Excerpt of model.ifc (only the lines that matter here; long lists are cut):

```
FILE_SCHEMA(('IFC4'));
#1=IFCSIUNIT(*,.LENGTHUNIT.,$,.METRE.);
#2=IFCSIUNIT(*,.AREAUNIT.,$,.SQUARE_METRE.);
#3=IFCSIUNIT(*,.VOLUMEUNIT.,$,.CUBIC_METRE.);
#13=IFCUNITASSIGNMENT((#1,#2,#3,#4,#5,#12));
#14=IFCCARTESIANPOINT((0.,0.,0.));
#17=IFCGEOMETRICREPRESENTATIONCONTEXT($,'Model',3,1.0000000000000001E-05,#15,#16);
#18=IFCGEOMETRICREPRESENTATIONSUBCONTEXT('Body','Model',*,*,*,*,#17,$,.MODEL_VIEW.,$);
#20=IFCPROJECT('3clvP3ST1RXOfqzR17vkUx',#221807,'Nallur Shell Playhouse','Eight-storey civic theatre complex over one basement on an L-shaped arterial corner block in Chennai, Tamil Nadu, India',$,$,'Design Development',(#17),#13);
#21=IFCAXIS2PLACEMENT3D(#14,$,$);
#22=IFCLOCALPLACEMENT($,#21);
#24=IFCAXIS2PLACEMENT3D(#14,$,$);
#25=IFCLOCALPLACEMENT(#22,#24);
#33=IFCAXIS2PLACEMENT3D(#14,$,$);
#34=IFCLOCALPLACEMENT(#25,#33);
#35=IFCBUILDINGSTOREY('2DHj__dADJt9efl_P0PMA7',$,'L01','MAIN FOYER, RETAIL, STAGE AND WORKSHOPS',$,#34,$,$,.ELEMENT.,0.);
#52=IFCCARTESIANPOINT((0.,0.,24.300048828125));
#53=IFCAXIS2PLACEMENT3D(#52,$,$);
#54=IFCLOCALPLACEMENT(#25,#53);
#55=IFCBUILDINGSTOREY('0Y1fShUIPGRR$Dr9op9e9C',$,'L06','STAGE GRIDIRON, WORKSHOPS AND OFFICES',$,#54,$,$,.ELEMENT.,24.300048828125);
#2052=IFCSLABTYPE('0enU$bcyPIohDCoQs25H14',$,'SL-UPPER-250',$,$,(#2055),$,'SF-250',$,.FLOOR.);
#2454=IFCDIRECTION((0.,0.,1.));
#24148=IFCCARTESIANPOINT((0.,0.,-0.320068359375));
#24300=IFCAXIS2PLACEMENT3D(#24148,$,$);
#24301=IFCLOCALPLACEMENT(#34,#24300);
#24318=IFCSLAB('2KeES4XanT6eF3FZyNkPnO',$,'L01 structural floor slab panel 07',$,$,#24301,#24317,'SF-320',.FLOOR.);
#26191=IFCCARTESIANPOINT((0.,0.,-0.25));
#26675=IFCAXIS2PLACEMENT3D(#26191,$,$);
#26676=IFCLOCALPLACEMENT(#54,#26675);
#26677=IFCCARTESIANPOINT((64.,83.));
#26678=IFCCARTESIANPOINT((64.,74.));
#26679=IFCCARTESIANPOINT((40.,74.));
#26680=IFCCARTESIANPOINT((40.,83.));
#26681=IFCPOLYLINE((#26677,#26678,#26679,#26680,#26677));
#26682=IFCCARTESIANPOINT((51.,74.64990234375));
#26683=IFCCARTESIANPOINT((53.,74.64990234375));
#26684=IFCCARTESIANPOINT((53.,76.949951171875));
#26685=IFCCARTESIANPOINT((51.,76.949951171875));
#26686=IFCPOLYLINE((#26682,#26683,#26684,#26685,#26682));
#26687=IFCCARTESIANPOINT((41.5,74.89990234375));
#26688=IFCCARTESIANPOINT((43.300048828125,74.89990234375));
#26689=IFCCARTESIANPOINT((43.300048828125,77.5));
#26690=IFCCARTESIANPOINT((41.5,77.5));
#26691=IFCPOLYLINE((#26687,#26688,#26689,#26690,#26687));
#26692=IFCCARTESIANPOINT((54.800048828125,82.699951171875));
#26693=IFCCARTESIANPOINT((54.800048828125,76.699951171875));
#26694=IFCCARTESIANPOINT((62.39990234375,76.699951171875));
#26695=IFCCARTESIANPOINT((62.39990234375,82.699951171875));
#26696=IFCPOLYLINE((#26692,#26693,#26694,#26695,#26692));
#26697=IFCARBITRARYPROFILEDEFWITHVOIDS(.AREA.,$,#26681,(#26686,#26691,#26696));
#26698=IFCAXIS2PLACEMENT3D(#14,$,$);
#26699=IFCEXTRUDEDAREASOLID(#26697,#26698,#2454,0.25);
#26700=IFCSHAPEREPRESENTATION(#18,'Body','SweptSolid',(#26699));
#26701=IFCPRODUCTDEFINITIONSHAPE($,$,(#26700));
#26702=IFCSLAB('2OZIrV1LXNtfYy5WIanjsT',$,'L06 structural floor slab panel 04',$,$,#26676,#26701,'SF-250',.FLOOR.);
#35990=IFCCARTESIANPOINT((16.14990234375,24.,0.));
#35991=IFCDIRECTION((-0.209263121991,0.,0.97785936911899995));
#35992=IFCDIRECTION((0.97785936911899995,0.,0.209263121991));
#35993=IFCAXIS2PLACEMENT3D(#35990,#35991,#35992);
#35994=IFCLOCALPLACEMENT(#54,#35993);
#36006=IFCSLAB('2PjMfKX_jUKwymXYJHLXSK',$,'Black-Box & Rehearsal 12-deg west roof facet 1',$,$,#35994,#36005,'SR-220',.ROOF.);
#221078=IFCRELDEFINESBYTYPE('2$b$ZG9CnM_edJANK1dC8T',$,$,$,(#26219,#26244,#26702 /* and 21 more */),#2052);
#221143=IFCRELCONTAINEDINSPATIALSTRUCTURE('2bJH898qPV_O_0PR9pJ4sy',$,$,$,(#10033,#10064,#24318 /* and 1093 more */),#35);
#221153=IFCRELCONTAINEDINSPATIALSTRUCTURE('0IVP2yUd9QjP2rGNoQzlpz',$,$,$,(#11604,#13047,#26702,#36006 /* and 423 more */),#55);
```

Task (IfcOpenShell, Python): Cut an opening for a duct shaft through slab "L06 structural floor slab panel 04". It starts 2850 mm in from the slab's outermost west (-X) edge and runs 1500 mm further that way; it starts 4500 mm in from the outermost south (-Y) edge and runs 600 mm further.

```python
import numpy as np
import ifcopenshell
import ifcopenshell.api.feature
import ifcopenshell.api.geometry
import ifcopenshell.api.root
import ifcopenshell.geom
import ifcopenshell.util.placement
import ifcopenshell.util.representation
import ifcopenshell.util.shape
import ifcopenshell.util.unit

model = ifcopenshell.open("model.ifc")
unit_scale = ifcopenshell.util.unit.calculate_unit_scale(model)
settings = ifcopenshell.geom.settings()


def volume(element):
    """Net volume in cubic metres, openings subtracted."""
    shape = ifcopenshell.geom.create_shape(settings, element)
    return ifcopenshell.util.shape.get_volume(shape.geometry)


slab = model.by_id(26702)
before = volume(slab)

# Extent in the slab's own axes, in metres. The edges named are its -X and -Y sides.
slab_shape = ifcopenshell.geom.create_shape(settings, slab)
vertices = ifcopenshell.util.shape.get_vertices(slab_shape.geometry)
x_min, y_min, bottom = vertices.min(axis=0)
top = vertices[:, 2].max()

opening = ifcopenshell.api.root.create_entity(model, ifc_class="IfcOpeningElement", name="Duct shaft opening", predefined_type="OPENING")
context = ifcopenshell.util.representation.get_context(model, "Model", "Body", "MODEL_VIEW")
width, depth = 1.5, 0.6
outline = [(0.0, 0.0), (width, 0.0), (width, depth), (0.0, depth), (0.0, 0.0)]
# Overshoot both faces by 50 mm so the cut is clean.
shape = ifcopenshell.api.geometry.add_slab_representation(
    model, context=context, depth=top - bottom + 0.1, polyline=outline
)
ifcopenshell.api.geometry.assign_representation(model, product=opening, representation=shape)

matrix = ifcopenshell.util.placement.get_local_placement(slab.ObjectPlacement)
matrix[:, 3] = matrix @ np.append(np.array([x_min + 2.85, y_min + 4.5, bottom - 0.05]) / unit_scale, 1.0)
ifcopenshell.api.geometry.edit_object_placement(model, product=opening, matrix=matrix, is_si=False)
ifcopenshell.api.feature.add_feature(model, feature=opening, element=slab)

after = volume(slab)

print(f"slab volume {before:.3f} -> {after:.3f} m3")

model.write("model-out.ifc")
```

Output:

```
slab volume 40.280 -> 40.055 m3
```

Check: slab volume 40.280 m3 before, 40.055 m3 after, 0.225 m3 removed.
